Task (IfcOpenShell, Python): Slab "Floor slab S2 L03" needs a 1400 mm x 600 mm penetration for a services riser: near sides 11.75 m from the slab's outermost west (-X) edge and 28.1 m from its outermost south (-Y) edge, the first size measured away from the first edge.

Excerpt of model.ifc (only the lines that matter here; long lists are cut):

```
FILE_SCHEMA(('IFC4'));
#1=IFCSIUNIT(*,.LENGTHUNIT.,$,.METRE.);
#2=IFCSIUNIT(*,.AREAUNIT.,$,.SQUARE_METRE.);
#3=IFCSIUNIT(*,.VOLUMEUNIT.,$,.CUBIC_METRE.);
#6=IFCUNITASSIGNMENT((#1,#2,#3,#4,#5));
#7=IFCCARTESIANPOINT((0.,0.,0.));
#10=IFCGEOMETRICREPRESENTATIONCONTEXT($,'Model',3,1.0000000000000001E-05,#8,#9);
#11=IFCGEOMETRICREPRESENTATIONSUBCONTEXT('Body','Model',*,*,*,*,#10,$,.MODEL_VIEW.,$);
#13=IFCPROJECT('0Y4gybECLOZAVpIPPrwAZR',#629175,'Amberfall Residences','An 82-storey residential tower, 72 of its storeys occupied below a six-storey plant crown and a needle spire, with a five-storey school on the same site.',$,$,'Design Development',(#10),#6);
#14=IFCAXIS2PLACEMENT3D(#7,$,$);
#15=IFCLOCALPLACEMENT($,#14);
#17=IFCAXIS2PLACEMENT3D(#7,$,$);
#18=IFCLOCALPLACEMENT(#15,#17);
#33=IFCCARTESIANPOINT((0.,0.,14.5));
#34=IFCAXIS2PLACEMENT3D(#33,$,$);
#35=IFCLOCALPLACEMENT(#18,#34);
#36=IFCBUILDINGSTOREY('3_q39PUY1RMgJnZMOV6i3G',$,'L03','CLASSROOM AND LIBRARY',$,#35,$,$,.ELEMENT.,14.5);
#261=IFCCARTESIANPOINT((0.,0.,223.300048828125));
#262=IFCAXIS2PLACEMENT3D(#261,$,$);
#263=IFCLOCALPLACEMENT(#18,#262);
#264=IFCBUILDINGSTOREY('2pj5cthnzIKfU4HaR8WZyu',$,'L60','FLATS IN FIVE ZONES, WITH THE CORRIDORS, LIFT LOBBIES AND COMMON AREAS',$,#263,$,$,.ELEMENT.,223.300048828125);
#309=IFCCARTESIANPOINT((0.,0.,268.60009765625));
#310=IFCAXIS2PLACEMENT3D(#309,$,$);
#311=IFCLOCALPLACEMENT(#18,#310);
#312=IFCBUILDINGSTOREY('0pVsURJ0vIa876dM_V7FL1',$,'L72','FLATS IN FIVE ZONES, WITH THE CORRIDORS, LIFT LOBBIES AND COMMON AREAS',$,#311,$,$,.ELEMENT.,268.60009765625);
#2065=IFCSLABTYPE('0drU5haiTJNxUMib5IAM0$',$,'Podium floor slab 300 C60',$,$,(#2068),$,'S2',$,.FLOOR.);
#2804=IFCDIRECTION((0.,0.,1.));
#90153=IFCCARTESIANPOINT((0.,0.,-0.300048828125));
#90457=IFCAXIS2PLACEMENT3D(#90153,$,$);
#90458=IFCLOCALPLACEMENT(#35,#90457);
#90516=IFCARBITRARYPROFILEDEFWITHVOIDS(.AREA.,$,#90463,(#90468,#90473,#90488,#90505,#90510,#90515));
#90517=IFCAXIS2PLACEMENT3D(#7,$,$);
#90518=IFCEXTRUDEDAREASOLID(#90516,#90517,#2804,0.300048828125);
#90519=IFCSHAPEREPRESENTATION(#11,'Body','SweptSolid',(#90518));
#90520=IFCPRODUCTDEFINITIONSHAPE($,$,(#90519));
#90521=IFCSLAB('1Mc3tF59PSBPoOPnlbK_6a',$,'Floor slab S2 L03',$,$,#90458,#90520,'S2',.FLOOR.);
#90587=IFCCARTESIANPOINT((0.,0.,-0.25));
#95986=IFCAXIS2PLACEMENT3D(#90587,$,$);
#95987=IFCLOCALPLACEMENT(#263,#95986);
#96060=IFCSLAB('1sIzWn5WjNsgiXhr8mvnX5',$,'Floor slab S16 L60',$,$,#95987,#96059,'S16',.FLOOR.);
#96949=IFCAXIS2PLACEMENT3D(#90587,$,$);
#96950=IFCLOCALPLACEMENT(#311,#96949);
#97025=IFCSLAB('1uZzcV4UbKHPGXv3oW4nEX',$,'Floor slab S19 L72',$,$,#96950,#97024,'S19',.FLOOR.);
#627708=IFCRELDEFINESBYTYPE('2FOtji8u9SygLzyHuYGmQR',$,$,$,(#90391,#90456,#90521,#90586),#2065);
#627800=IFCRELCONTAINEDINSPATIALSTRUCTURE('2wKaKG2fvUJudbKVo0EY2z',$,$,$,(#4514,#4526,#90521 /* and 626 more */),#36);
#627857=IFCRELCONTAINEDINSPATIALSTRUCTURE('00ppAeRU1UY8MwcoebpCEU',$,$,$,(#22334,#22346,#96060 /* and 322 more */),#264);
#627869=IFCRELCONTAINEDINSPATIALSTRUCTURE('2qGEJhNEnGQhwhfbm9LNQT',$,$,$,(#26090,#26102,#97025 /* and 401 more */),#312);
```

```python
import numpy as np
import ifcopenshell
import ifcopenshell.api.feature
import ifcopenshell.api.geometry
import ifcopenshell.api.root
import ifcopenshell.geom
import ifcopenshell.util.placement
import ifcopenshell.util.representation
import ifcopenshell.util.shape
import ifcopenshell.util.unit

model = ifcopenshell.open("model.ifc")
unit_scale = ifcopenshell.util.unit.calculate_unit_scale(model)
settings = ifcopenshell.geom.settings()


def volume(element):
    """Net volume in cubic metres, openings subtracted."""
    shape = ifcopenshell.geom.create_shape(settings, element)
    return ifcopenshell.util.shape.get_volume(shape.geometry)


slab = model.by_id(90521)
before = volume(slab)

# Extent in the slab's own axes, in metres. The edges named are its -X and -Y sides.
slab_shape = ifcopenshell.geom.create_shape(settings, slab)
vertices = ifcopenshell.util.shape.get_vertices(slab_shape.geometry)
x_min, y_min, bottom = vertices.min(axis=0)
top = vertices[:, 2].max()

opening = ifcopenshell.api.root.create_entity(model, ifc_class="IfcOpeningElement", name="Services riser opening", predefined_type="OPENING")
context = ifcopenshell.util.representation.get_context(model, "Model", "Body", "MODEL_VIEW")
width, depth = 1.4, 0.6
outline = [(0.0, 0.0), (width, 0.0), (width, depth), (0.0, depth), (0.0, 0.0)]
# Overshoot both faces by 50 mm so the cut is clean.
shape = ifcopenshell.api.geometry.add_slab_representation(
    model, context=context, depth=top - bottom + 0.1, polyline=outline
)
ifcopenshell.api.geometry.assign_representation(model, product=opening, representation=shape)

matrix = ifcopenshell.util.placement.get_local_placement(slab.ObjectPlacement)
matrix[:, 3] = matrix @ np.append(np.array([x_min + 11.75, y_min + 28.1, bottom - 0.05]) / unit_scale, 1.0)
ifcopenshell.api.geometry.edit_object_placement(model, product=opening, matrix=matrix, is_si=False)
ifcopenshell.api.feature.add_feature(model, feature=opening, element=slab)

after = volume(slab)

print(f"slab volume {before:.3f} -> {after:.3f} m3")

model.write("model-out.ifc")
```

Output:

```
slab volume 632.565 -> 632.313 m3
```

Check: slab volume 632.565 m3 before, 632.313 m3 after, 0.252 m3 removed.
